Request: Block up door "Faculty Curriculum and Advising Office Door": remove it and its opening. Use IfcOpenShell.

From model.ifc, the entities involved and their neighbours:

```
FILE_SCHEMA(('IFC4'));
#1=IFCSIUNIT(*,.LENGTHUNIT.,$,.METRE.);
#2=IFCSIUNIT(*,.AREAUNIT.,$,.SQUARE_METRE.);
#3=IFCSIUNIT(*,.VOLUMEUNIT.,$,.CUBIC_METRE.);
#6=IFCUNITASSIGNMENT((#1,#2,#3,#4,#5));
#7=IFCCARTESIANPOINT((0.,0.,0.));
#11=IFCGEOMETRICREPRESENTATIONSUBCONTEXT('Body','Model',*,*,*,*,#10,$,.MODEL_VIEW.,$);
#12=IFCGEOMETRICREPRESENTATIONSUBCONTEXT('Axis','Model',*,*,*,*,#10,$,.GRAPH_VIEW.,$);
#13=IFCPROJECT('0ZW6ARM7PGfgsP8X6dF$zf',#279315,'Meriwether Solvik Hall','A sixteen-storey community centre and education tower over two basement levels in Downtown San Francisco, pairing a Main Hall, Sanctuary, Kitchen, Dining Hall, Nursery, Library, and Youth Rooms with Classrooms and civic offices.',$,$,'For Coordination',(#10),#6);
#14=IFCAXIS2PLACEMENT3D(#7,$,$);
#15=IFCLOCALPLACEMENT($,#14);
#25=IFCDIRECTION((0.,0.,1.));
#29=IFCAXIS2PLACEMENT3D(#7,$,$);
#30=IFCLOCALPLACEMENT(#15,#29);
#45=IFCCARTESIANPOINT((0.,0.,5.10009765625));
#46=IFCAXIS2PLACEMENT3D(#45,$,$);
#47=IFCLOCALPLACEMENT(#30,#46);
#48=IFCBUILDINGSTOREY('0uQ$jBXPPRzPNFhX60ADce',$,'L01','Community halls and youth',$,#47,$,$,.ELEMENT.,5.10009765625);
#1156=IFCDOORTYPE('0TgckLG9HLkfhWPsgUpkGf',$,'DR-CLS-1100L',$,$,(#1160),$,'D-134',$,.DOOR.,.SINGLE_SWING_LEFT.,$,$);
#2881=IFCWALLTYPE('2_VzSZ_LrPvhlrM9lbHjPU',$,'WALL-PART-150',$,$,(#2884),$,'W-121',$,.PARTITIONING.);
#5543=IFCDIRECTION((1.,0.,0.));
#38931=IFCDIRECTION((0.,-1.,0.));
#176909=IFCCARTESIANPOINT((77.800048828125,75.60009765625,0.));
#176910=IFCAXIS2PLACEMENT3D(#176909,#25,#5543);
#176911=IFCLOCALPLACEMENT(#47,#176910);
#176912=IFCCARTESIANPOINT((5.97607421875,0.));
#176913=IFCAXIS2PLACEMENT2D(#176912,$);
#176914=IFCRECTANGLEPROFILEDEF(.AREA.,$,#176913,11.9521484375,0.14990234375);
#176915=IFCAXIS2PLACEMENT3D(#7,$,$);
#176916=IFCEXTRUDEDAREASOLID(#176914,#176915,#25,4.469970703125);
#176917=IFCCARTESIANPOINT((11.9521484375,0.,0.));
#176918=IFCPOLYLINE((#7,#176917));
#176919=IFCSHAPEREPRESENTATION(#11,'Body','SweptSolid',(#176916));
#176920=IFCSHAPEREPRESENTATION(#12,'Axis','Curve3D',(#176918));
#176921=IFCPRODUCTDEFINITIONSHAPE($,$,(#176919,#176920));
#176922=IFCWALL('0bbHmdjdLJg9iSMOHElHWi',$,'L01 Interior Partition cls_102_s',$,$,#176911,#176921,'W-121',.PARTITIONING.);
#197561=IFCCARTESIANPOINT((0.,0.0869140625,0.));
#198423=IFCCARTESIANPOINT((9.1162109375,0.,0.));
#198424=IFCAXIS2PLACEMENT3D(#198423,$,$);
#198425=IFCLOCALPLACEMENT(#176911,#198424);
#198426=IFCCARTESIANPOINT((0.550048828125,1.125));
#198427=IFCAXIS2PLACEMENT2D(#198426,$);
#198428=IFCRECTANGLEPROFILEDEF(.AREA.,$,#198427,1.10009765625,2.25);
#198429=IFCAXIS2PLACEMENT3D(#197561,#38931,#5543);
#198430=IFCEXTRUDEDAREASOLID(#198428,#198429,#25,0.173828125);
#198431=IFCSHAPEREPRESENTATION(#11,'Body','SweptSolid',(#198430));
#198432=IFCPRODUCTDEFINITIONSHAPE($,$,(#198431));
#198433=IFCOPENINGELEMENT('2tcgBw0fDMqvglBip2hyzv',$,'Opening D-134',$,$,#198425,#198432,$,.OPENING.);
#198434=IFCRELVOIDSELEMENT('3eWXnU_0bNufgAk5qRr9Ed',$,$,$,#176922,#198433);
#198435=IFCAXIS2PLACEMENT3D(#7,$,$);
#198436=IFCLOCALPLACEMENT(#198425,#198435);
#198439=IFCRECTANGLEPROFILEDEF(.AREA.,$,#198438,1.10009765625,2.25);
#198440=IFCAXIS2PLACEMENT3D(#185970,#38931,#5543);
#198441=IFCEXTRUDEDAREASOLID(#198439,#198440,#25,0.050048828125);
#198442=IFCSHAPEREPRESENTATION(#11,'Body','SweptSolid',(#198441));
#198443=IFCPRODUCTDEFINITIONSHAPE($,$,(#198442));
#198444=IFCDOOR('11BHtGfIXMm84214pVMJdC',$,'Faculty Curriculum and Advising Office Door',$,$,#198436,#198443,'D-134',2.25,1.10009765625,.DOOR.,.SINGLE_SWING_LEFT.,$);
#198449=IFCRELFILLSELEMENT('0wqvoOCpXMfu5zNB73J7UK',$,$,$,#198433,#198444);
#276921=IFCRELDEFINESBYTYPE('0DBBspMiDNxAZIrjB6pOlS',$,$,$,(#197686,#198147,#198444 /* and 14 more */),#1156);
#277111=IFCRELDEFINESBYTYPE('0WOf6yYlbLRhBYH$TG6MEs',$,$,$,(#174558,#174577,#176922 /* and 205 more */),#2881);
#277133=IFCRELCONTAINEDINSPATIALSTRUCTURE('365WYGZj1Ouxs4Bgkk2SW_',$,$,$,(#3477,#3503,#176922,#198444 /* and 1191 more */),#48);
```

```python
import ifcopenshell
import ifcopenshell.api.feature
import ifcopenshell.api.root
import ifcopenshell.geom
import ifcopenshell.util.shape

model = ifcopenshell.open("model.ifc")
settings = ifcopenshell.geom.settings()


def volume(element):
    """Net volume in cubic metres, openings subtracted."""
    shape = ifcopenshell.geom.create_shape(settings, element)
    return ifcopenshell.util.shape.get_volume(shape.geometry)


door = model.by_guid("11BHtGfIXMm84214pVMJdC")
opening = door.FillsVoids[0].RelatingOpeningElement
wall = opening.VoidsElements[0].RelatingBuildingElement
before = volume(wall)

ifcopenshell.api.root.remove_product(model, product=door)
ifcopenshell.api.feature.remove_feature(model, feature=opening)

after = volume(wall)

print(f"wall volume {before:.3f} -> {after:.3f} m3")

model.write("model_rev.ifc")
```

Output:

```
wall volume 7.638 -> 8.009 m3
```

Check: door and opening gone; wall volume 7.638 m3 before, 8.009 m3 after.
